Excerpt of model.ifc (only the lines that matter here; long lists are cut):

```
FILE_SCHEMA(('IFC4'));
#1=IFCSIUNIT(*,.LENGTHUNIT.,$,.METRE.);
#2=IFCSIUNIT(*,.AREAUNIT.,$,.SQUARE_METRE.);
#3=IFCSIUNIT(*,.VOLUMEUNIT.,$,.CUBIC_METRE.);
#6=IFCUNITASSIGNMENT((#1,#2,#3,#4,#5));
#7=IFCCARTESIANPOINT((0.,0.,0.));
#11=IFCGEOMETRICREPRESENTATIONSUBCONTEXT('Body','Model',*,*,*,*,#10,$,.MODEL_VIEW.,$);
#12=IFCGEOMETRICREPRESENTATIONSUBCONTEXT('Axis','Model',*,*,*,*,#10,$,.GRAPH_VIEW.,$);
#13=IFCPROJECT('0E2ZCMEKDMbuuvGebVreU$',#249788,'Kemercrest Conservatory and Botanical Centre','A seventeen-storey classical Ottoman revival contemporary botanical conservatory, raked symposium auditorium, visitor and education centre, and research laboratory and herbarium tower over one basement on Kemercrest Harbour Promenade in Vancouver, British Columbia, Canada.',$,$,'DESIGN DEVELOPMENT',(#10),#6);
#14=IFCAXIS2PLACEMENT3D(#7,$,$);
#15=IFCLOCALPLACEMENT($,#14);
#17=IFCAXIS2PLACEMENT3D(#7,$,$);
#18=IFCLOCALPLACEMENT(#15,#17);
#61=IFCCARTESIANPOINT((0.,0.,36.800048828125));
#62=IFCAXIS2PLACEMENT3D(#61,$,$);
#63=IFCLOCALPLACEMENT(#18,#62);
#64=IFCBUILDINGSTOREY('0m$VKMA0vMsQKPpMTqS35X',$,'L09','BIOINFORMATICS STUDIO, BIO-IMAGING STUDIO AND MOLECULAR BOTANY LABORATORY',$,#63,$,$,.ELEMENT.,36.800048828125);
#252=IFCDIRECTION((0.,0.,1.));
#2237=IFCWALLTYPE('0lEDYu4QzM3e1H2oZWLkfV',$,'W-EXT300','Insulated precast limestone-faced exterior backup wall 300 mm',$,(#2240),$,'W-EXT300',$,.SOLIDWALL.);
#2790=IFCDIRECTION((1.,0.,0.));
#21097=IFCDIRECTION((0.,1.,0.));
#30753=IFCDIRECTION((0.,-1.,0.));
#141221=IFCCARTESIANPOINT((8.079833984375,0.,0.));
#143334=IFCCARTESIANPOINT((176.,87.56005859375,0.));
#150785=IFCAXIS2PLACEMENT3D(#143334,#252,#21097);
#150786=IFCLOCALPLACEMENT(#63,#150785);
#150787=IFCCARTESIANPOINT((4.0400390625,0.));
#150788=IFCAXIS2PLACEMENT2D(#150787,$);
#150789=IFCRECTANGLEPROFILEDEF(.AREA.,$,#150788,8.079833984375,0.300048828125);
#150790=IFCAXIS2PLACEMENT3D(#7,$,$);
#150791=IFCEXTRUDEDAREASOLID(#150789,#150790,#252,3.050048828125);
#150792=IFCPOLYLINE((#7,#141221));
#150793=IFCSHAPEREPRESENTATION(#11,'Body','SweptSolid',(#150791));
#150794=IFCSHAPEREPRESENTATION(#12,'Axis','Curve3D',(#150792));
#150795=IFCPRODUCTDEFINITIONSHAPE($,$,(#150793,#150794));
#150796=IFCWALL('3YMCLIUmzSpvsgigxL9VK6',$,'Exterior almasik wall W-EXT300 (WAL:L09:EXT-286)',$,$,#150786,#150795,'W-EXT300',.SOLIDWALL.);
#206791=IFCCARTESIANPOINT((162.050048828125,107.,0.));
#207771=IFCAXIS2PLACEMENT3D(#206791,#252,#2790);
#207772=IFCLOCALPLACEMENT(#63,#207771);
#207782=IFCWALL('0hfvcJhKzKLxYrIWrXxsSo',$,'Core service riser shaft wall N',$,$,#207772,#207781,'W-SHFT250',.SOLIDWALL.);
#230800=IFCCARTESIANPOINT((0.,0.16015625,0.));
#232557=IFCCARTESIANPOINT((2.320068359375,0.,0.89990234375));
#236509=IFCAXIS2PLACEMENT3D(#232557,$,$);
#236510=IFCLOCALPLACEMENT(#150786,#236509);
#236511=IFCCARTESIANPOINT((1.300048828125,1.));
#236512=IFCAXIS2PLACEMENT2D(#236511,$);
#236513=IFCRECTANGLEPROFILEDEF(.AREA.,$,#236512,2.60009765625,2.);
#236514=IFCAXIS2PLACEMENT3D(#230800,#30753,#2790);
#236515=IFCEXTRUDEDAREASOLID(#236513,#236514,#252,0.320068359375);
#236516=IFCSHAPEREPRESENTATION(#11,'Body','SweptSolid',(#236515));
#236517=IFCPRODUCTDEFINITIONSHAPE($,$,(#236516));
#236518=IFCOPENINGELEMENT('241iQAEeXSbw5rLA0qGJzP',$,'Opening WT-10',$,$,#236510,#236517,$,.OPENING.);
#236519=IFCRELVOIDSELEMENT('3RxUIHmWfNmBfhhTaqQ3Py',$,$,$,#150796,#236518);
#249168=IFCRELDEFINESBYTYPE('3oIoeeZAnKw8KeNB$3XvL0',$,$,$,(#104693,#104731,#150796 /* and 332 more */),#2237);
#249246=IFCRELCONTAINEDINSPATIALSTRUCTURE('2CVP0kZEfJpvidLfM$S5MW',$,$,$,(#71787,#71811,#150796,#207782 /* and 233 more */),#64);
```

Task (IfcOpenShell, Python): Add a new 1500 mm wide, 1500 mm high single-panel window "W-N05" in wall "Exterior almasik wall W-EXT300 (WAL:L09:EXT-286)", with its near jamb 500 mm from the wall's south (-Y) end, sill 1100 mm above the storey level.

```python
import numpy as np
import ifcopenshell
import ifcopenshell.api.feature
import ifcopenshell.api.geometry
import ifcopenshell.api.root
import ifcopenshell.api.spatial
import ifcopenshell.geom
import ifcopenshell.util.element
import ifcopenshell.util.placement
import ifcopenshell.util.representation
import ifcopenshell.util.shape
import ifcopenshell.util.unit

model = ifcopenshell.open("model.ifc")
unit_scale = ifcopenshell.util.unit.calculate_unit_scale(model)
settings = ifcopenshell.geom.settings()


def volume(element):
    """Net volume in cubic metres, openings subtracted."""
    shape = ifcopenshell.geom.create_shape(settings, element)
    return ifcopenshell.util.shape.get_volume(shape.geometry)


wall = model.by_guid("3YMCLIUmzSpvsgigxL9VK6")
storey = ifcopenshell.util.element.get_container(wall, ifc_class="IfcBuildingStorey")
context = ifcopenshell.util.representation.get_context(model, "Model", "Body", "MODEL_VIEW")
before = volume(wall)

width, height, from_end, sill = 1.5, 1.5, 0.5, 1.1  # metres

# The wall runs along its own X axis, and the end named is its -X end.
wall_shape = ifcopenshell.geom.create_shape(settings, wall)
x, y, z = ifcopenshell.util.shape.get_vertices(wall_shape.geometry).T
start = x.min() + from_end
face, thickness = float(y.min()), float(y.max() - y.min())
wall_matrix = ifcopenshell.util.placement.get_local_placement(wall.ObjectPlacement)
level = ifcopenshell.util.placement.get_local_placement(storey.ObjectPlacement)[2, 3]


def in_wall(x, y):
    """Placement at x, y metres in the wall's axes, at sill height."""
    matrix = wall_matrix.copy()
    matrix[:, 3] = wall_matrix @ np.array([x / unit_scale, y / unit_scale, 0.0, 1.0])
    matrix[2, 3] = level + sill / unit_scale
    return matrix


# Opening: a box that overshoots both wall faces by 50 mm.
opening = ifcopenshell.api.root.create_entity(model, ifc_class="IfcOpeningElement", predefined_type="OPENING")
box = ifcopenshell.api.geometry.add_wall_representation(
    model, context=context, length=width, height=height, thickness=thickness + 0.1
)
ifcopenshell.api.geometry.assign_representation(model, product=opening, representation=box)
ifcopenshell.api.geometry.edit_object_placement(model, product=opening, matrix=in_wall(start, face - 0.05), is_si=False)
ifcopenshell.api.feature.add_feature(model, feature=opening, element=wall)

window = ifcopenshell.api.root.create_entity(model, ifc_class="IfcWindow", name="W-N05", predefined_type="WINDOW")
window.OverallWidth, window.OverallHeight = width / unit_scale, height / unit_scale
window.PartitioningType = "SINGLE_PANEL"
body = ifcopenshell.api.geometry.add_window_representation(
    model,
    context=context,
    overall_width=window.OverallWidth,
    overall_height=window.OverallHeight,
    partition_type="SINGLE_PANEL",
)
ifcopenshell.api.geometry.assign_representation(model, product=window, representation=body)
ifcopenshell.api.spatial.assign_container(model, products=[window], relating_structure=storey)
ifcopenshell.api.feature.add_filling(model, opening=opening, element=window)

# Centre the window in the wall's thickness.
ifcopenshell.api.geometry.edit_object_placement(model, product=window, matrix=in_wall(start, face), is_si=False)
window_shape = ifcopenshell.geom.create_shape(settings, window)
depth = ifcopenshell.util.shape.get_vertices(window_shape.geometry)[:, 1]
offset = face + thickness / 2 - (depth.min() + depth.max()) / 2
ifcopenshell.api.geometry.edit_object_placement(model, product=window, matrix=in_wall(start, offset), is_si=False)

after = volume(wall)

print(f"wall volume {before:.3f} -> {after:.3f} m3")

model.write("model_edited.ifc")
```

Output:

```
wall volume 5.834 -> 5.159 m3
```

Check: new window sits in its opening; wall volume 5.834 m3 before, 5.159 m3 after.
